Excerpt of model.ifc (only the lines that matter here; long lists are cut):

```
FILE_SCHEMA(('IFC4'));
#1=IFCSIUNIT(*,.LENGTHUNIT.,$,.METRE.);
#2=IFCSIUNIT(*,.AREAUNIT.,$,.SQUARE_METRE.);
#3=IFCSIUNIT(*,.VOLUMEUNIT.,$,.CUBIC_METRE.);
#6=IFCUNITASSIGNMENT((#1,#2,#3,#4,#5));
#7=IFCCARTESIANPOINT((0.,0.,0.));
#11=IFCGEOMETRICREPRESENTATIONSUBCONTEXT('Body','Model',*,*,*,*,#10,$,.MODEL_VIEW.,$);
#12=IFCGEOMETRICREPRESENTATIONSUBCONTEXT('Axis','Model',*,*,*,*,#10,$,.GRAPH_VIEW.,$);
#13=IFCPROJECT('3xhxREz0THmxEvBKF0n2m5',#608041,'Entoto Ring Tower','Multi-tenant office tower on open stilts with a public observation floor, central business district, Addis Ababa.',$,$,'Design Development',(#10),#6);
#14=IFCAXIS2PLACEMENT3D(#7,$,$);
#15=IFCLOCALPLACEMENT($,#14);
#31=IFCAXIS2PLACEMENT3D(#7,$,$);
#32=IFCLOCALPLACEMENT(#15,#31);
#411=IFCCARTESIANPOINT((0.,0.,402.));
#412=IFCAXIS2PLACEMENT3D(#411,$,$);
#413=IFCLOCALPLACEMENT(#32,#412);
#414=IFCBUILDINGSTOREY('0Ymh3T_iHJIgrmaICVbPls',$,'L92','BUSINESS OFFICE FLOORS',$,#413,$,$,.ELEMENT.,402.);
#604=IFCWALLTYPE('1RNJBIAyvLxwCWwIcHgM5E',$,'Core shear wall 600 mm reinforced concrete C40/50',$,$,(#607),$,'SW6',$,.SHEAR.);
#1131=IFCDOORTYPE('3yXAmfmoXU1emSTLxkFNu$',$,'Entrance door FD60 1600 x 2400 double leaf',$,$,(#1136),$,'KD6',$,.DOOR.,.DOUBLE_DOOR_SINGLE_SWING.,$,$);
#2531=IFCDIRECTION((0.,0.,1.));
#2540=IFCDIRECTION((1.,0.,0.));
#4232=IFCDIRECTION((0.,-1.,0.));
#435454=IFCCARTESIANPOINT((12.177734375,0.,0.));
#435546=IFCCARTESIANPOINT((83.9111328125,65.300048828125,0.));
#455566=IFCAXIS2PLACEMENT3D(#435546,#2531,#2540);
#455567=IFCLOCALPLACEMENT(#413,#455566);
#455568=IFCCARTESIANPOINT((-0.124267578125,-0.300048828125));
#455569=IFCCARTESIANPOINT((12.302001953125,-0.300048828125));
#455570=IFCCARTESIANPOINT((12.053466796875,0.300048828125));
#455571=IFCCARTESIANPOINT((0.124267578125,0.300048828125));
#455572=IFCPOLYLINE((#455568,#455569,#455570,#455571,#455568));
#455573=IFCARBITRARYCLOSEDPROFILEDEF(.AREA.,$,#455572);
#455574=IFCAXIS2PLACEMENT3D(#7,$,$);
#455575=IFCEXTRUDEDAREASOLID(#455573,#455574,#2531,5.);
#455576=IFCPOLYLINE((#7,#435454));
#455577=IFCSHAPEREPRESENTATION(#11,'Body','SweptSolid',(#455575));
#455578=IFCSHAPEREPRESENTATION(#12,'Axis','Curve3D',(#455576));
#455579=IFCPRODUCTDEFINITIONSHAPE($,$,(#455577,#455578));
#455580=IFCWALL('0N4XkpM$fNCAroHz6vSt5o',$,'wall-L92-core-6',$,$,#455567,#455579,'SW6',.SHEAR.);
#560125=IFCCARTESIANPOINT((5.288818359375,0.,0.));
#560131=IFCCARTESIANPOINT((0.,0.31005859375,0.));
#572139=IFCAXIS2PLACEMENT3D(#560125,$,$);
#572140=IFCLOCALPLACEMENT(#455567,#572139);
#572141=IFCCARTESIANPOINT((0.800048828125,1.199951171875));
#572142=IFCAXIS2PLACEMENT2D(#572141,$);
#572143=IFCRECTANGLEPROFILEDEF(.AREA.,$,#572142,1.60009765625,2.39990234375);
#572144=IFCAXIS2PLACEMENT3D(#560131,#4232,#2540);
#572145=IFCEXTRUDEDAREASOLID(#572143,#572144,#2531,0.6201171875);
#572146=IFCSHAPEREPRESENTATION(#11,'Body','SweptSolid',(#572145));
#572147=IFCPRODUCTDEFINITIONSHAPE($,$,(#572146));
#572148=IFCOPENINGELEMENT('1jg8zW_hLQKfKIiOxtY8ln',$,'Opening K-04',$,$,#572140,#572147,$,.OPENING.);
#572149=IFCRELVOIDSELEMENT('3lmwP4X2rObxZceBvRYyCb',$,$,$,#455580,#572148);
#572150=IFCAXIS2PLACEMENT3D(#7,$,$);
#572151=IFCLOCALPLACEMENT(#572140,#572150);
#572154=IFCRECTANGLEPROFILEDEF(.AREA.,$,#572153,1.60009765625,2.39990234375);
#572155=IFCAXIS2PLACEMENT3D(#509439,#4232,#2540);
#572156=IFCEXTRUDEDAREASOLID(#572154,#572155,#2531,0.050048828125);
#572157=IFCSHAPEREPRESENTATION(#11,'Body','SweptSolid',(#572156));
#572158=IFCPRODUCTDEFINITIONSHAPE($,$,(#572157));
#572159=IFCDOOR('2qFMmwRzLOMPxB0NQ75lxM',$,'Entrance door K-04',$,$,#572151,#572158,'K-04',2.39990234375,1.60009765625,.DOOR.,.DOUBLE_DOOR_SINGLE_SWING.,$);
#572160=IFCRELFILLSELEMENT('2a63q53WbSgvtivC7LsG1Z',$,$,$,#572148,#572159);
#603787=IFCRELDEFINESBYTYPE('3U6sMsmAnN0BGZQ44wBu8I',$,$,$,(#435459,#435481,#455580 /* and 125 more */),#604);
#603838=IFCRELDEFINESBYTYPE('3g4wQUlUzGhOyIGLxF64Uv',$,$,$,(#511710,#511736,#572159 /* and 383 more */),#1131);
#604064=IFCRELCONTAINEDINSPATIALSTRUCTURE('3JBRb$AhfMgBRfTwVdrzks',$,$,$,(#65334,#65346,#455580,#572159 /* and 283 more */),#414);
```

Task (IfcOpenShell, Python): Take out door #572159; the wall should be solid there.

```python
import ifcopenshell
import ifcopenshell.api.feature
import ifcopenshell.api.root
import ifcopenshell.geom
import ifcopenshell.util.shape

model = ifcopenshell.open("model.ifc")
settings = ifcopenshell.geom.settings()


def volume(element):
    """Net volume in cubic metres, openings subtracted."""
    shape = ifcopenshell.geom.create_shape(settings, element)
    return ifcopenshell.util.shape.get_volume(shape.geometry)


door = model.by_guid("2qFMmwRzLOMPxB0NQ75lxM")
opening = door.FillsVoids[0].RelatingOpeningElement
wall = opening.VoidsElements[0].RelatingBuildingElement
before = volume(wall)

ifcopenshell.api.root.remove_product(model, product=door)
ifcopenshell.api.feature.remove_feature(model, feature=opening)

after = volume(wall)

print(f"wall volume {before:.3f} -> {after:.3f} m3")

model.write("model_edited.ifc")
```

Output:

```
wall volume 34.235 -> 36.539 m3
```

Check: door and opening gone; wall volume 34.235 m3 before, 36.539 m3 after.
